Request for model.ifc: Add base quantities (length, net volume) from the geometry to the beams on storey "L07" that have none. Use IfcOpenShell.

First a look at what the model holds.

```python
import ifcopenshell
import ifcopenshell.util.element
import ifcopenshell.util.unit

model = ifcopenshell.open("model.ifc")
print(model.schema)
for unit_type in ("LENGTHUNIT", "AREAUNIT", "VOLUMEUNIT"):
    print(unit_type, ifcopenshell.util.unit.calculate_unit_scale(model, unit_type))
storey = next(s for s in model.by_type("IfcBuildingStorey") if s.Name == "L07")
beams = [e for e in ifcopenshell.util.element.get_decomposition(storey) if e.is_a("IfcBeam")]
for e in sorted(beams, key=lambda e: e.id()):
    print(e.id(), e.is_a(), e.Name, list(ifcopenshell.util.element.get_psets(e, qtos_only=True)), sep=" | ")
```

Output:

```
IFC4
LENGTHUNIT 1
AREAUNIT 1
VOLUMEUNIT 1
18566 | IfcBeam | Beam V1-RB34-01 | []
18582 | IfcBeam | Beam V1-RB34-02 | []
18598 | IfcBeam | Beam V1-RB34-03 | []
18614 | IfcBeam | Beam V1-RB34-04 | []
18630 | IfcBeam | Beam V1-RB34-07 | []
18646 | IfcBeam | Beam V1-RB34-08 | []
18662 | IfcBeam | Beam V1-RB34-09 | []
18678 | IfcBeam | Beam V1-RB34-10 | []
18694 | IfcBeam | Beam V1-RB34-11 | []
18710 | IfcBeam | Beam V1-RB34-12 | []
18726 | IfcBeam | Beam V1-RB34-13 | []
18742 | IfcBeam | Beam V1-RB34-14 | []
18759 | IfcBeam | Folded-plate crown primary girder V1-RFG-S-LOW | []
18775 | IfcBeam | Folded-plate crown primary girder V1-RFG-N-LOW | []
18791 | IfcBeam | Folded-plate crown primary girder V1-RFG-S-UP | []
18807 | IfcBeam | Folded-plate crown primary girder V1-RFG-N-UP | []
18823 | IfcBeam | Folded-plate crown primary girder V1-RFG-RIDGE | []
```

```python
import ifcopenshell
import ifcopenshell.api.pset
import ifcopenshell.geom
import ifcopenshell.util.element
import ifcopenshell.util.shape
import ifcopenshell.util.unit

model = ifcopenshell.open("model.ifc")
unit_scale = ifcopenshell.util.unit.calculate_unit_scale(model)
volume_scale = ifcopenshell.util.unit.calculate_unit_scale(model, "VOLUMEUNIT")
settings = ifcopenshell.geom.settings()

storey = next(s for s in model.by_type("IfcBuildingStorey") if s.Name == "L07")
beams = [e for e in ifcopenshell.util.element.get_decomposition(storey) if e.is_a("IfcBeam")]

for e in sorted(beams, key=lambda e: e.id()):
    if ifcopenshell.util.element.get_psets(e, qtos_only=True, should_inherit=False):
        continue
    # Geometry comes back in metres, in the element's own axes.
    shape = ifcopenshell.geom.create_shape(settings, e)
    values = {
        "Length": ifcopenshell.util.shape.get_max_xyz(shape.geometry) / unit_scale,
        "NetVolume": ifcopenshell.util.shape.get_volume(shape.geometry) / volume_scale,
    }
    qto = ifcopenshell.api.pset.add_qto(model, product=e, name="Qto_BeamBaseQuantities")
    ifcopenshell.api.pset.edit_qto(model, qto=qto, properties=values)
    print(e.id(), {k: round(v, 3) for k, v in values.items()})

model.write("model_rev.ifc")
```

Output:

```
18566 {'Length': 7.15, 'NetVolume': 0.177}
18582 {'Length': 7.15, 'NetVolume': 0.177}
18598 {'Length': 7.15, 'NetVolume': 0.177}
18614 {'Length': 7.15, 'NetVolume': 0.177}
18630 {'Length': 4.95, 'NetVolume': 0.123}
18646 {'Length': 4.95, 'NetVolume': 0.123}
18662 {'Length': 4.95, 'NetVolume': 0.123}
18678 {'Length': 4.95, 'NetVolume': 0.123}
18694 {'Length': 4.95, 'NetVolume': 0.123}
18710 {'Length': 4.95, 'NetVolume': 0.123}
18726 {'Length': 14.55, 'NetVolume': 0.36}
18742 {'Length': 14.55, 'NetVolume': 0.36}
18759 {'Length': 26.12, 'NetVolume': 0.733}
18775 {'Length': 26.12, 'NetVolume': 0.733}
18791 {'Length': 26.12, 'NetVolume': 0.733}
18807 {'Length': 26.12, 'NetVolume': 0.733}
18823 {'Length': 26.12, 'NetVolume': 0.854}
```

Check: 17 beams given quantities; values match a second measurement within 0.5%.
